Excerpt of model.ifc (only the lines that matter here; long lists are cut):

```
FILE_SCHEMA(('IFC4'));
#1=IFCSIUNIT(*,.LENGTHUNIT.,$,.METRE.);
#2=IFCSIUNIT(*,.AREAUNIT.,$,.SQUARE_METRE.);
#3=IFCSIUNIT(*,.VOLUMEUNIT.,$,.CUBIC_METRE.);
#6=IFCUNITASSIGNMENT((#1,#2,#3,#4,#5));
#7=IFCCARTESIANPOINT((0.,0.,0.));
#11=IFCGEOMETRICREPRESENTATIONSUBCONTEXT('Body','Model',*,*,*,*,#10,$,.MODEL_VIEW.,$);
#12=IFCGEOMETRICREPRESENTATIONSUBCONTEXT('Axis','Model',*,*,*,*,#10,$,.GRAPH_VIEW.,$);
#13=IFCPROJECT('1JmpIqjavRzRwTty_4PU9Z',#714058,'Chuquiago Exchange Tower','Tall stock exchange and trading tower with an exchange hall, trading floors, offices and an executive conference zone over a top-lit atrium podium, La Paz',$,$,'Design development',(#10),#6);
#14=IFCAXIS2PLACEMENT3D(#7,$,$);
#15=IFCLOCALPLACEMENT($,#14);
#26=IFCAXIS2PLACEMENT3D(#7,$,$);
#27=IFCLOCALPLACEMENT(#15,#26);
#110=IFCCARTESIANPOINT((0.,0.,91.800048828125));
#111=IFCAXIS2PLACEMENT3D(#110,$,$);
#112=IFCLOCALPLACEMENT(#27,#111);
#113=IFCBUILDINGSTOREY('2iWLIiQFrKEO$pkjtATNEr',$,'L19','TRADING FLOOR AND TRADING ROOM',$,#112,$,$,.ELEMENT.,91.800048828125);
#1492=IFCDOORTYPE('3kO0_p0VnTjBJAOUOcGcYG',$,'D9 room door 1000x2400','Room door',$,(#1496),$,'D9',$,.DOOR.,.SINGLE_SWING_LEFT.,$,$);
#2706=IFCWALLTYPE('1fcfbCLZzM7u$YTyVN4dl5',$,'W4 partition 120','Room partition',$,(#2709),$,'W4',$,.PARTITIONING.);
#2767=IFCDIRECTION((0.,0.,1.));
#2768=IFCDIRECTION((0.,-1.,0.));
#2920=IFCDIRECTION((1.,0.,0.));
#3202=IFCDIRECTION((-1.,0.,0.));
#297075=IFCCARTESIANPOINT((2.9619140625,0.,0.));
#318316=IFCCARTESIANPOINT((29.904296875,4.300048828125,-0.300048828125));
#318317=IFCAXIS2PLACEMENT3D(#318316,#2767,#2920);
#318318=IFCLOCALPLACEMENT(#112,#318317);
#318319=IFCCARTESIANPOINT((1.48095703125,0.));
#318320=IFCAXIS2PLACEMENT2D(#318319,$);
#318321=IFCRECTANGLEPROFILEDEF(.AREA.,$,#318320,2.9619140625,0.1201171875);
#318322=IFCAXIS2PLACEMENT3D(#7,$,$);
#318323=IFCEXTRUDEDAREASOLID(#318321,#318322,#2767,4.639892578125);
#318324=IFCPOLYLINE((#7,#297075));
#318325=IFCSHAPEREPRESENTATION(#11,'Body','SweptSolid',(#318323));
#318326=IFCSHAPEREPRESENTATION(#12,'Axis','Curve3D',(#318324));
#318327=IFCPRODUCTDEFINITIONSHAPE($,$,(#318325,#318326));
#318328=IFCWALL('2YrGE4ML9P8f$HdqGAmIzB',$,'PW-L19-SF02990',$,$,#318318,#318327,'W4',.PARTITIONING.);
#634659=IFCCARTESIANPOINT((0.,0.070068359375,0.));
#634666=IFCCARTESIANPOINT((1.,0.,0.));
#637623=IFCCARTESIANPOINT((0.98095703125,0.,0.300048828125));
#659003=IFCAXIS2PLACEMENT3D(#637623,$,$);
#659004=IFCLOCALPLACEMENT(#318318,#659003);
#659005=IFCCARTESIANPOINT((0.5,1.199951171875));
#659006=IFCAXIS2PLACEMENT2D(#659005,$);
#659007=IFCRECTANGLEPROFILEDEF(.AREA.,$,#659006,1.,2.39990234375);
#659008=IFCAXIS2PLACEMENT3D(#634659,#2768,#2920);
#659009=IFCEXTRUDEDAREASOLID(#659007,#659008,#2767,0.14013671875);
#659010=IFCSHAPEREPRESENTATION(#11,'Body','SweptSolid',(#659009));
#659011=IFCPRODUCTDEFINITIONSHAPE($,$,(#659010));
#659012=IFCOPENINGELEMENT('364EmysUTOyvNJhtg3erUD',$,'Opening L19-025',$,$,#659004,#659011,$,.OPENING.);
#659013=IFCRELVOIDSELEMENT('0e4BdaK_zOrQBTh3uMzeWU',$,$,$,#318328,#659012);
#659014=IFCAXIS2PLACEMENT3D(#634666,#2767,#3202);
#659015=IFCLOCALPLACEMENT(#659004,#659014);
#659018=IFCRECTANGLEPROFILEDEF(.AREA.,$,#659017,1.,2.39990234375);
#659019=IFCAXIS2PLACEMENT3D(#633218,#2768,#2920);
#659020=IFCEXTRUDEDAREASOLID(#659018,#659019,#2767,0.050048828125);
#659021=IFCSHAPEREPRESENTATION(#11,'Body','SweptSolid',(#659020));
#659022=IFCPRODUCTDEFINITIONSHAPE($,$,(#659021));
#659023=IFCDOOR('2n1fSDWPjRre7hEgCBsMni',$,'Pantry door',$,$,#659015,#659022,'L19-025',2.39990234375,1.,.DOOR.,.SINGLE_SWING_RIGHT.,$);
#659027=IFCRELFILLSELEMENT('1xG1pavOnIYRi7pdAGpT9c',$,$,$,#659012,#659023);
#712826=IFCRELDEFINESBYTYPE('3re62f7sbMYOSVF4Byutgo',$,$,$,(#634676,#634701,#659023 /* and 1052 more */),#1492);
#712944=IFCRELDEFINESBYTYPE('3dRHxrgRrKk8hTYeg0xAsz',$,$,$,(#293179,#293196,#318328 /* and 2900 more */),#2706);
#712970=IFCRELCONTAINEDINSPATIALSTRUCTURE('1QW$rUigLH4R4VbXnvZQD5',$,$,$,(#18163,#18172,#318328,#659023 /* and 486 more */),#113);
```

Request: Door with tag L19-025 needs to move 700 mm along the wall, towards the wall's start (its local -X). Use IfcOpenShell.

```python
import ifcopenshell
import ifcopenshell.api.geometry
import ifcopenshell.util.placement

model = ifcopenshell.open("model.ifc")

door = model.by_id(659023)
opening = door.FillsVoids[0].RelatingOpeningElement
wall = opening.VoidsElements[0].RelatingBuildingElement

wall_matrix = ifcopenshell.util.placement.get_local_placement(wall.ObjectPlacement)
shift = wall_matrix[:3, 0] * -0.7
before = ifcopenshell.util.placement.get_local_placement(door.ObjectPlacement)[:3, 3].copy()

# The door is placed relative to its opening, so it follows when the opening moves.
matrix = ifcopenshell.util.placement.get_local_placement(opening.ObjectPlacement)
matrix[:3, 3] += shift
ifcopenshell.api.geometry.edit_object_placement(
    model, product=opening, matrix=matrix, is_si=False, should_transform_children=True
)

after = ifcopenshell.util.placement.get_local_placement(door.ObjectPlacement)[:3, 3]
print("door moved by", (after - before).round(3) + 0.0)

model.write("model-out.ifc")
```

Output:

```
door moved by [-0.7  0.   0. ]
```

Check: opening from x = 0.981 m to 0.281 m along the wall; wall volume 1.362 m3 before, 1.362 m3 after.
